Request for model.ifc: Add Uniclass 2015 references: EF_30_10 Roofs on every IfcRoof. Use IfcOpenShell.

First a look at what the model holds.

```python
import ifcopenshell

model = ifcopenshell.open("model.ifc")
print(model.schema)
print("classifications:", [c.Name for c in model.by_type("IfcClassification")])
for ifc_class in ("IfcDoor", "IfcRoof", "IfcStair", "IfcWall", "IfcWindow"):
    print(ifc_class, len(model.by_type(ifc_class)))
```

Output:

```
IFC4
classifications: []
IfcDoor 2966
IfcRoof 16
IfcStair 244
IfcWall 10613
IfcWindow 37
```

```python
import ifcopenshell
import ifcopenshell.api.classification

model = ifcopenshell.open("model.ifc")

system = ifcopenshell.api.classification.add_classification(model, classification="Uniclass 2015")

codes = {
    "IfcRoof": ("EF_30_10", "Roofs"),
}
for ifc_class, (code, name) in codes.items():
    products = model.by_type(ifc_class)
    ifcopenshell.api.classification.add_reference(
        model, products=products, classification=system, identification=code, name=name
    )
    print(code, len(products))

model.write("model_updated.ifc")
```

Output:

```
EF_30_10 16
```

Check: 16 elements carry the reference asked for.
